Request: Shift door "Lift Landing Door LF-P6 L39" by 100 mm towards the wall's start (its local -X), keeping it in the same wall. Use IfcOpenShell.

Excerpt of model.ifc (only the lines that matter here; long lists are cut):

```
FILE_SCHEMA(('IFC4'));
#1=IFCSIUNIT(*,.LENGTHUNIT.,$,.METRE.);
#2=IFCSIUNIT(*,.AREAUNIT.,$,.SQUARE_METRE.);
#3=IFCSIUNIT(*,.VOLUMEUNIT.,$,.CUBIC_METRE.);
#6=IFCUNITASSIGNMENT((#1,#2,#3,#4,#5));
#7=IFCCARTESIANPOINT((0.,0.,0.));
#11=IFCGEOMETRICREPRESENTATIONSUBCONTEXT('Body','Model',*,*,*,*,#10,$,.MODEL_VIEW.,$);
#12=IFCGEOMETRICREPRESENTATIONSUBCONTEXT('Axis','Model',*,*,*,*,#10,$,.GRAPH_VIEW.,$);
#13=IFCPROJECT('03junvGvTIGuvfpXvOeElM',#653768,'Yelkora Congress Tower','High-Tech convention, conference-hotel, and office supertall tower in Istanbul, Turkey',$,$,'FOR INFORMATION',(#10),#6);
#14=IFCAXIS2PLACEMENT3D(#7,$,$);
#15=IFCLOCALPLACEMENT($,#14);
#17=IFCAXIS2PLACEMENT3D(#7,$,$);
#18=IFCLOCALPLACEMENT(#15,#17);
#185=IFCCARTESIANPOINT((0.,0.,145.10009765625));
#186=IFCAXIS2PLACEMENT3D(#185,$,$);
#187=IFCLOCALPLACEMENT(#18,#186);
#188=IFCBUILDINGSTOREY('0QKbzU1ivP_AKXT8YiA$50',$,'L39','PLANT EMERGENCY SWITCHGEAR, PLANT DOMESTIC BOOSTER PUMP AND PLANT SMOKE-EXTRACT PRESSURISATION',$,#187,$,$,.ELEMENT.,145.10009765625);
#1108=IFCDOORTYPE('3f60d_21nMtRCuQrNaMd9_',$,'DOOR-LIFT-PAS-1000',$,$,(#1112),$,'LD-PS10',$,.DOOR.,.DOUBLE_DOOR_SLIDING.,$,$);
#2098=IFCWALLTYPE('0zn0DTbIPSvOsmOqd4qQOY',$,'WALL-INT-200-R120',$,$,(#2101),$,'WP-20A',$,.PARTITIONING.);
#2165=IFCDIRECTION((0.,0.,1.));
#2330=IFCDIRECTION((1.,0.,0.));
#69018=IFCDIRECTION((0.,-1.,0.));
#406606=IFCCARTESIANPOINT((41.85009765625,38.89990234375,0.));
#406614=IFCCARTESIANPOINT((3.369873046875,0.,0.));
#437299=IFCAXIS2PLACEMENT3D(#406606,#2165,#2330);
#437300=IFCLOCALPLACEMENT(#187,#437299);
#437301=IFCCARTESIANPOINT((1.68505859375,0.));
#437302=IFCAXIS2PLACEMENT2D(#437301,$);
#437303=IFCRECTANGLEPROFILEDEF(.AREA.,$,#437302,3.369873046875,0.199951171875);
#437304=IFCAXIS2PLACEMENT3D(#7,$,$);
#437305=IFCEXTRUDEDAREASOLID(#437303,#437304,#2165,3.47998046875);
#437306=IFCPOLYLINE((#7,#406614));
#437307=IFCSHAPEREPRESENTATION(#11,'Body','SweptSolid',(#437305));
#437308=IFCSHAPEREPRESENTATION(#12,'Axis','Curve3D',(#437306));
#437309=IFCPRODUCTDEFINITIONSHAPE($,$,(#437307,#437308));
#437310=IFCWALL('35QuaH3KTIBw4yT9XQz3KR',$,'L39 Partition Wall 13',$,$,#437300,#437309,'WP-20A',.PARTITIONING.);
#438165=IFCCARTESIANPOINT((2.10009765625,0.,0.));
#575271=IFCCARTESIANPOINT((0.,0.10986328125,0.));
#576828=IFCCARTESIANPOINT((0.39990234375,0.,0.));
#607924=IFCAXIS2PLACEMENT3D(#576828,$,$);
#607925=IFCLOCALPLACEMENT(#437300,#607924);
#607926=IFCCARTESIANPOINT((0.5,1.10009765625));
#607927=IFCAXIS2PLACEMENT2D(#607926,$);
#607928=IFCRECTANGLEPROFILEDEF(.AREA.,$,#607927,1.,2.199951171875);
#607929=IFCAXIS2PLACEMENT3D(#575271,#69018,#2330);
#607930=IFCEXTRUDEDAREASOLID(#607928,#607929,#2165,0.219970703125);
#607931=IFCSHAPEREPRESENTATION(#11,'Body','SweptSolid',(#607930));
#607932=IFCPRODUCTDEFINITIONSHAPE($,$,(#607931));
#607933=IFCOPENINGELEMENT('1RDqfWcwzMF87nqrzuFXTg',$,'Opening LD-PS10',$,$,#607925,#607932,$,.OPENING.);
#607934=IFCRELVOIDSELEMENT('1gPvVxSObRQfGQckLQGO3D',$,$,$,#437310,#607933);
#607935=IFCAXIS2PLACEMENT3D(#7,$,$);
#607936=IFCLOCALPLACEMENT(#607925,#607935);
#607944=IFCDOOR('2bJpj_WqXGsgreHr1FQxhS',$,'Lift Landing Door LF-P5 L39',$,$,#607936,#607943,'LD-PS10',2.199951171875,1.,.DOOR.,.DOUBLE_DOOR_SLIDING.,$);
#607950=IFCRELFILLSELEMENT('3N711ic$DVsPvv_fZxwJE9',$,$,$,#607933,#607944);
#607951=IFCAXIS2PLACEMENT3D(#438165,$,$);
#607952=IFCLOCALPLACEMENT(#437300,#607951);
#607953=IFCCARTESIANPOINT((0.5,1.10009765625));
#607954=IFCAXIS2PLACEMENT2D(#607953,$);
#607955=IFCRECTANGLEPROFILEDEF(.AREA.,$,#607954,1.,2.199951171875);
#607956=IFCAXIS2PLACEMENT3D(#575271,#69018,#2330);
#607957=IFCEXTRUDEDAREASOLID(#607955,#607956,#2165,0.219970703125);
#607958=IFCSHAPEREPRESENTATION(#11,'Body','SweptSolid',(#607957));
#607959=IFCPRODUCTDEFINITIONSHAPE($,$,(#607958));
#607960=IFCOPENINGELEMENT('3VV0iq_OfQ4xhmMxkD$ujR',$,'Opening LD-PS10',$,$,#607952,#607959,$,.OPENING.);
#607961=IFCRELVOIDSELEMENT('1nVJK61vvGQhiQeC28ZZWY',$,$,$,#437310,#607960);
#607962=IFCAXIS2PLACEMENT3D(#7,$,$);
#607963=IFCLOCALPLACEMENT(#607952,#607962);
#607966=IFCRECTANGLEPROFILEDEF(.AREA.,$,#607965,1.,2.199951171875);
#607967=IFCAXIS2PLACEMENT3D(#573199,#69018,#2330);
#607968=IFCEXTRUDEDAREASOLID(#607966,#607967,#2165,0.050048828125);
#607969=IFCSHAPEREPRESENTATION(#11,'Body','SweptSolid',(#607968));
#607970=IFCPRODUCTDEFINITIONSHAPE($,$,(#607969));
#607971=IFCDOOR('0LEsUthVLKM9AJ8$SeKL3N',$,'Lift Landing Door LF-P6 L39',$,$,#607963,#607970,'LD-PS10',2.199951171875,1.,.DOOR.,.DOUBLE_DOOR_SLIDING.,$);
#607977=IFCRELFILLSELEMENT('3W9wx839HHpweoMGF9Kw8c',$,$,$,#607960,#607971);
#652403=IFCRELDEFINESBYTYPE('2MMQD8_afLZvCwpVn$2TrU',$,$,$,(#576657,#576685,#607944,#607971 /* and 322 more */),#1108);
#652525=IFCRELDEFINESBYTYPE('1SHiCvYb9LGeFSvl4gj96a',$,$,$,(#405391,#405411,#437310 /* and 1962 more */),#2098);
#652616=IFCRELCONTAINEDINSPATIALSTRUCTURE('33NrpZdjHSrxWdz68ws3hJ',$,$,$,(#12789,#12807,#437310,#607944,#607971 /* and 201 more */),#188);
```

```python
import ifcopenshell
import ifcopenshell.api.geometry
import ifcopenshell.util.placement
import ifcopenshell.util.unit

model = ifcopenshell.open("model.ifc")
unit_scale = ifcopenshell.util.unit.calculate_unit_scale(model)

door = model.by_guid("0LEsUthVLKM9AJ8$SeKL3N")
opening = door.FillsVoids[0].RelatingOpeningElement
wall = opening.VoidsElements[0].RelatingBuildingElement

wall_matrix = ifcopenshell.util.placement.get_local_placement(wall.ObjectPlacement)
shift = wall_matrix[:3, 0] * -0.1 / unit_scale
before = ifcopenshell.util.placement.get_local_placement(door.ObjectPlacement)[:3, 3].copy()

# The door is placed relative to its opening, so it follows when the opening moves.
matrix = ifcopenshell.util.placement.get_local_placement(opening.ObjectPlacement)
matrix[:3, 3] += shift
ifcopenshell.api.geometry.edit_object_placement(
    model, product=opening, matrix=matrix, is_si=False, should_transform_children=True
)

after = ifcopenshell.util.placement.get_local_placement(door.ObjectPlacement)[:3, 3]
print("door moved by", (after - before).round(3) + 0.0)

model.write("model-out.ifc")
```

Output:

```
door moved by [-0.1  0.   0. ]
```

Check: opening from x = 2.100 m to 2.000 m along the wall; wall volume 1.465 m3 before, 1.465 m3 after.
